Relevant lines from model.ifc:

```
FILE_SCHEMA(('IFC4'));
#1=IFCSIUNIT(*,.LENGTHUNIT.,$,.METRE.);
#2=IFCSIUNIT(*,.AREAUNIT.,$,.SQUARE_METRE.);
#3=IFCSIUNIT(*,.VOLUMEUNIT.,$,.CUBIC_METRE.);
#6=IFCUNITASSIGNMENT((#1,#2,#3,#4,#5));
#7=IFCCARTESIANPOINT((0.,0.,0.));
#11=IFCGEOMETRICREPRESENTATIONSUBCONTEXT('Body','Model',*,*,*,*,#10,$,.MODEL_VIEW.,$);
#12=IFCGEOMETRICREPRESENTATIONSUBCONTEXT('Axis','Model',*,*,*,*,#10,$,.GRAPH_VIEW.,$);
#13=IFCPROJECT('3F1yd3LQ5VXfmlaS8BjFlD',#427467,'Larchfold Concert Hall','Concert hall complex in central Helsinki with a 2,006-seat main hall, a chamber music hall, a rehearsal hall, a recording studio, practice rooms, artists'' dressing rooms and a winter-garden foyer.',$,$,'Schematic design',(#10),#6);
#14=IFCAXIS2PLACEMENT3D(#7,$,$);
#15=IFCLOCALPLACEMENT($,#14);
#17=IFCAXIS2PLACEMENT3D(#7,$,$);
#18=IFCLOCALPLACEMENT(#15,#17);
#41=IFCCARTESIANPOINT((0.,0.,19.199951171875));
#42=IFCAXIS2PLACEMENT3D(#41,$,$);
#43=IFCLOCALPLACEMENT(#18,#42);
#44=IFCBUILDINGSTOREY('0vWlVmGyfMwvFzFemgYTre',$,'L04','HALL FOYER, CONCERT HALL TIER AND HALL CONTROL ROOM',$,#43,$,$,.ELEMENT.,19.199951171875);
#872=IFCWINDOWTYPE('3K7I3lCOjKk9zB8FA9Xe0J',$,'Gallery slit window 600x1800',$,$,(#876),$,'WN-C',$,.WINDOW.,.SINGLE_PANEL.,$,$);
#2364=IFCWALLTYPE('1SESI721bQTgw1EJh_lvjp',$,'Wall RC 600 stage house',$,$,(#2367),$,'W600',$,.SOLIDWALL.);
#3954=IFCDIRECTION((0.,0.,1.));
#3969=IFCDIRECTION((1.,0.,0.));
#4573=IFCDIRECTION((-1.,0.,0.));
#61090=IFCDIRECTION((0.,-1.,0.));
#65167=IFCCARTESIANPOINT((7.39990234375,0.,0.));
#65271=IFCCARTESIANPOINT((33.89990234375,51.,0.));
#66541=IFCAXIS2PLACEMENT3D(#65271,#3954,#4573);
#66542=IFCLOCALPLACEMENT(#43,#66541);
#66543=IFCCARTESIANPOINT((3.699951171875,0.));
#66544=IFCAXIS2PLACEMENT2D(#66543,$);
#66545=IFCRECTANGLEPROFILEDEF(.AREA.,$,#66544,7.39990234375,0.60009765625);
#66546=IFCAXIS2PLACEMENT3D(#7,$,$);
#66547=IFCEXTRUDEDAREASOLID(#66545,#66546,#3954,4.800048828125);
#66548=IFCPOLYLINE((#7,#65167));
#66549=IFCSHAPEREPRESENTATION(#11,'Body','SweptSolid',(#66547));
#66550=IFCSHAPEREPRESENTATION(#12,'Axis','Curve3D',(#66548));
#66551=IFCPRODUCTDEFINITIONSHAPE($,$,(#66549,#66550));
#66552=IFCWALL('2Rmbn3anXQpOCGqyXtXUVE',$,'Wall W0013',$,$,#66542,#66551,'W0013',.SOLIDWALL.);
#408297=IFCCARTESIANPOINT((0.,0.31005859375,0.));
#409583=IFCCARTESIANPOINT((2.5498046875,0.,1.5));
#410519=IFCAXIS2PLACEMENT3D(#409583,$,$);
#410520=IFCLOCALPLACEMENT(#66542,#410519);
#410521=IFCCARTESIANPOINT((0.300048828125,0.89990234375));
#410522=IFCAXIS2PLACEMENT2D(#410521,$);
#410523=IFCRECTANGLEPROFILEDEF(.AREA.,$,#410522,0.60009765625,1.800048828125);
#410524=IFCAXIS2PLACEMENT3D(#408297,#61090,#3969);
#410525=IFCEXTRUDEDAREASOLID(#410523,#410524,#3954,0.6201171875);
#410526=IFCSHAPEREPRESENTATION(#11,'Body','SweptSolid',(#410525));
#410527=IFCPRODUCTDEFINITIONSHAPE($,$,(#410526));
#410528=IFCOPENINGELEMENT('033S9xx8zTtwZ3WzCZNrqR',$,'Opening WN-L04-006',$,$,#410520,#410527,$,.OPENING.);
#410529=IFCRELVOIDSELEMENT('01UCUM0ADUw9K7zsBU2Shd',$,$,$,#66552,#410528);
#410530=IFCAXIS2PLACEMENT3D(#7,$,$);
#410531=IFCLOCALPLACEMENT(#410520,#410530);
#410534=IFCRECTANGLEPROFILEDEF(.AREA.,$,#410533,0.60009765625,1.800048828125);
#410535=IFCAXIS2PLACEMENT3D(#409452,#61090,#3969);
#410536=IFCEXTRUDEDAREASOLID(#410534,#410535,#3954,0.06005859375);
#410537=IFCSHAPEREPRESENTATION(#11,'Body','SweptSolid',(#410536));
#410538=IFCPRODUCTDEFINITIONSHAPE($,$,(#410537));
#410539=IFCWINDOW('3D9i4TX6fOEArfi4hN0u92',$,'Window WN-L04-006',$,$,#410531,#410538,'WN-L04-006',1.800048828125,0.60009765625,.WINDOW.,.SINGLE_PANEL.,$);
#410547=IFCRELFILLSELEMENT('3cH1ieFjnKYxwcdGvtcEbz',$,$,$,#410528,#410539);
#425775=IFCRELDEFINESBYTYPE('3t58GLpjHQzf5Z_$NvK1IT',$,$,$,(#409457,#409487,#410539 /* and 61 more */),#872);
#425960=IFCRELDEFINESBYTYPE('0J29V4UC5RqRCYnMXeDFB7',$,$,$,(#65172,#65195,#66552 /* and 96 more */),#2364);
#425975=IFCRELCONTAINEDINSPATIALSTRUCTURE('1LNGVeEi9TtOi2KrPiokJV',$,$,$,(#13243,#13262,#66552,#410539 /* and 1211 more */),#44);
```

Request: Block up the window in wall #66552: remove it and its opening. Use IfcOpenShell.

```python
import ifcopenshell
import ifcopenshell.api.feature
import ifcopenshell.api.root
import ifcopenshell.geom
import ifcopenshell.util.shape

model = ifcopenshell.open("model.ifc")
settings = ifcopenshell.geom.settings()


def volume(element):
    """Net volume in cubic metres, openings subtracted."""
    shape = ifcopenshell.geom.create_shape(settings, element)
    return ifcopenshell.util.shape.get_volume(shape.geometry)


window = model.by_guid("3D9i4TX6fOEArfi4hN0u92")
opening = window.FillsVoids[0].RelatingOpeningElement
wall = opening.VoidsElements[0].RelatingBuildingElement
before = volume(wall)

ifcopenshell.api.root.remove_product(model, product=window)
ifcopenshell.api.feature.remove_feature(model, feature=opening)

after = volume(wall)

print(f"wall volume {before:.3f} -> {after:.3f} m3")

model.write("model_rev.ifc")
```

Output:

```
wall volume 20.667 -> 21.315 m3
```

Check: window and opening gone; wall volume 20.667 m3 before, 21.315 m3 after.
